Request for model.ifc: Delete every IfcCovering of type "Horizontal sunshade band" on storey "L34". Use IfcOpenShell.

First a look at what the model holds.

```python
import ifcopenshell
import ifcopenshell.util.element

model = ifcopenshell.open("model.ifc")
print(model.schema)
storey = next(s for s in model.by_type("IfcBuildingStorey") if s.Name == "L34")
coverings = [e for e in ifcopenshell.util.element.get_decomposition(storey) if e.is_a("IfcCovering")]
seen = {}
for e in coverings:
    element_type = ifcopenshell.util.element.get_type(e)
    name = element_type.Name if element_type not in (None, e) else None
    seen[name] = seen.get(name, 0) + 1
for name, count in sorted(seen.items(), key=str):
    print(count, "x", name)
```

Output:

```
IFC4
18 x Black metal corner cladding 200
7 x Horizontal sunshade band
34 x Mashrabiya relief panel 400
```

```python
import ifcopenshell
import ifcopenshell.api.root
import ifcopenshell.util.element

model = ifcopenshell.open("model.ifc")

storey = next(s for s in model.by_type("IfcBuildingStorey") if s.Name == "L34")
coverings = [e for e in ifcopenshell.util.element.get_decomposition(storey) if e.is_a("IfcCovering")]
targets = [e for e in coverings if (t := ifcopenshell.util.element.get_type(e)) not in (None, e) and t.Name == "Horizontal sunshade band"]

for e in targets:
    ifcopenshell.api.root.remove_product(model, product=e)
print(len(targets), "removed")

model.write("model_rev.ifc")
```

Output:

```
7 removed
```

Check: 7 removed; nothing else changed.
